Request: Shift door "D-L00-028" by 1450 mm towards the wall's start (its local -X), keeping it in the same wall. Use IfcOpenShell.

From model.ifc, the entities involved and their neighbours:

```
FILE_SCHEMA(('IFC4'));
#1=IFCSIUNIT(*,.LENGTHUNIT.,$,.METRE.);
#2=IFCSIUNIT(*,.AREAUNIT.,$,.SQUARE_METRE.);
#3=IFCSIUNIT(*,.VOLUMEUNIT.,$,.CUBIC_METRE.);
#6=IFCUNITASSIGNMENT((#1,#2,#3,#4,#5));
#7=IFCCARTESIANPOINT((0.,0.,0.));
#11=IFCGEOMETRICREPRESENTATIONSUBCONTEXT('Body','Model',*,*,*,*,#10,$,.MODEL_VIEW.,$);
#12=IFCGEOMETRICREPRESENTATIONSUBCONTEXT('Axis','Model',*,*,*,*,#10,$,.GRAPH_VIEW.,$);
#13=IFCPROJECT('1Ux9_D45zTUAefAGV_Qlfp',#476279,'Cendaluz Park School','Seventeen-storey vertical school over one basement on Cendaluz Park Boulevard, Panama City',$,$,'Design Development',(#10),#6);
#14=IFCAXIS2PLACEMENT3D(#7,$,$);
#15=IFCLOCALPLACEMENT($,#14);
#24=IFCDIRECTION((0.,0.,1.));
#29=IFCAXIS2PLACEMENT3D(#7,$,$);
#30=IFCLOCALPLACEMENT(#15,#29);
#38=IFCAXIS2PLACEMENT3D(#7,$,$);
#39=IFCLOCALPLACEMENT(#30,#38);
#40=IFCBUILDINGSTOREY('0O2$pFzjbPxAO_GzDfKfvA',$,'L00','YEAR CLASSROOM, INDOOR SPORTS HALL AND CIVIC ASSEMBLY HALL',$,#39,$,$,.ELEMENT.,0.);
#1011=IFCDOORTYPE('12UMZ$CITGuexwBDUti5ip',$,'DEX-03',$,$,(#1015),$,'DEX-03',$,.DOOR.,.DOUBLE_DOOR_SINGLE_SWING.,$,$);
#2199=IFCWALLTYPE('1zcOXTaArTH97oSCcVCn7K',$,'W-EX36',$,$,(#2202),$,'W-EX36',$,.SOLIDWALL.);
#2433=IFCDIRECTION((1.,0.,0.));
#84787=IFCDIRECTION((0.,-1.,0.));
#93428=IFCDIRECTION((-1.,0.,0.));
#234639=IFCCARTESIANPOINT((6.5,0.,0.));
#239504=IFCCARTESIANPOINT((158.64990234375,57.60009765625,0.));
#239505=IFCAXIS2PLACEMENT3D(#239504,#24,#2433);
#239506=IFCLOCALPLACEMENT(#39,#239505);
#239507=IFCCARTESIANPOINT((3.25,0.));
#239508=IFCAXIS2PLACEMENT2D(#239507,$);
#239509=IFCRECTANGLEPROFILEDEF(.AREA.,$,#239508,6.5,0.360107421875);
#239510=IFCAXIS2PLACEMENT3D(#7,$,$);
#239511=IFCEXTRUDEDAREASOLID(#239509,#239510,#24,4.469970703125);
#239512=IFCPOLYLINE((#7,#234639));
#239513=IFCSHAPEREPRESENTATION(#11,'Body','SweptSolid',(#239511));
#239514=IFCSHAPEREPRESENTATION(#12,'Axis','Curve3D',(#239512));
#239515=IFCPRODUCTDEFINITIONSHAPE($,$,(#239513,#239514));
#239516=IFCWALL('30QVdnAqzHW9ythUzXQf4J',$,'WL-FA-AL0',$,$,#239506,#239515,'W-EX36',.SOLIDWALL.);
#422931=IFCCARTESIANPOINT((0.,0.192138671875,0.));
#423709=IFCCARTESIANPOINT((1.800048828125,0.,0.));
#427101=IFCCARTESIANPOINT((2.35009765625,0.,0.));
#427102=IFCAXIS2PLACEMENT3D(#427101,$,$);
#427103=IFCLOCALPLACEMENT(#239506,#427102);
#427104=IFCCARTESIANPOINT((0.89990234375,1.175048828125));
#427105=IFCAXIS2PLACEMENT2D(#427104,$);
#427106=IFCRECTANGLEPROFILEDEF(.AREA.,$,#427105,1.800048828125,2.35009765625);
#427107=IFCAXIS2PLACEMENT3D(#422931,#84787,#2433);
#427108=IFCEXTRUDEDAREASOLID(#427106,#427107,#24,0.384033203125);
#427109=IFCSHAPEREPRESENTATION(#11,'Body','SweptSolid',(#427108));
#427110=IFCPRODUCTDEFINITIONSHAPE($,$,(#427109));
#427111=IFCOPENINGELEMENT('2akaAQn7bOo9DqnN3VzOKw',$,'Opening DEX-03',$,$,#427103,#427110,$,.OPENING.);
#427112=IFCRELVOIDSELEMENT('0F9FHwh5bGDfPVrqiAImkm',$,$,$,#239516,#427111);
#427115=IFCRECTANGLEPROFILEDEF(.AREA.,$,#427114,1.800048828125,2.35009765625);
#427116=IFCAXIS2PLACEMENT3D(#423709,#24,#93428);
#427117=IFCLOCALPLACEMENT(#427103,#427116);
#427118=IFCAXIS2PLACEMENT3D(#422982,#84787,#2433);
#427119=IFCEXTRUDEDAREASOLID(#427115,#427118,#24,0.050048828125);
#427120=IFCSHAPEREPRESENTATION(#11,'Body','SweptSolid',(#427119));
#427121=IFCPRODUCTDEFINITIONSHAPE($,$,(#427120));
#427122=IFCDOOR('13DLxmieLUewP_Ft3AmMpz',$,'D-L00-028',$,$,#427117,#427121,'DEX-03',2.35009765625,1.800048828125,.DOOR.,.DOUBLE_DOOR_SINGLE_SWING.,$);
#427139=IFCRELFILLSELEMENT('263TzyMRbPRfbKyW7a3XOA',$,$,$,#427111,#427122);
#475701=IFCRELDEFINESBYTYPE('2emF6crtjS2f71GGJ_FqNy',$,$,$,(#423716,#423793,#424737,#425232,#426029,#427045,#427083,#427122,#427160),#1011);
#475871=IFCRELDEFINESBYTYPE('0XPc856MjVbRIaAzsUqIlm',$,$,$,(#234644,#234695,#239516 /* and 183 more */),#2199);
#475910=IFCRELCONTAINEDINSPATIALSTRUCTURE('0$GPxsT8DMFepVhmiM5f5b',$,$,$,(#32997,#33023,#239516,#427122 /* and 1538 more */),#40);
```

```python
import ifcopenshell
import ifcopenshell.api.geometry
import ifcopenshell.util.placement
import ifcopenshell.util.unit

model = ifcopenshell.open("model.ifc")
unit_scale = ifcopenshell.util.unit.calculate_unit_scale(model)

door = model.by_guid("13DLxmieLUewP_Ft3AmMpz")
opening = door.FillsVoids[0].RelatingOpeningElement
wall = opening.VoidsElements[0].RelatingBuildingElement

wall_matrix = ifcopenshell.util.placement.get_local_placement(wall.ObjectPlacement)
shift = wall_matrix[:3, 0] * -1.45 / unit_scale
before = ifcopenshell.util.placement.get_local_placement(door.ObjectPlacement)[:3, 3].copy()

# The door is placed relative to its opening, so it follows when the opening moves.
matrix = ifcopenshell.util.placement.get_local_placement(opening.ObjectPlacement)
matrix[:3, 3] += shift
ifcopenshell.api.geometry.edit_object_placement(
    model, product=opening, matrix=matrix, is_si=False, should_transform_children=True
)

after = ifcopenshell.util.placement.get_local_placement(door.ObjectPlacement)[:3, 3]
print("door moved by", (after - before).round(3) + 0.0)

model.write("model_v2.ifc")
```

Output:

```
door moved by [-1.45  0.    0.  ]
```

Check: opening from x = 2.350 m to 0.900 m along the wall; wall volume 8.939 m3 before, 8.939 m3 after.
